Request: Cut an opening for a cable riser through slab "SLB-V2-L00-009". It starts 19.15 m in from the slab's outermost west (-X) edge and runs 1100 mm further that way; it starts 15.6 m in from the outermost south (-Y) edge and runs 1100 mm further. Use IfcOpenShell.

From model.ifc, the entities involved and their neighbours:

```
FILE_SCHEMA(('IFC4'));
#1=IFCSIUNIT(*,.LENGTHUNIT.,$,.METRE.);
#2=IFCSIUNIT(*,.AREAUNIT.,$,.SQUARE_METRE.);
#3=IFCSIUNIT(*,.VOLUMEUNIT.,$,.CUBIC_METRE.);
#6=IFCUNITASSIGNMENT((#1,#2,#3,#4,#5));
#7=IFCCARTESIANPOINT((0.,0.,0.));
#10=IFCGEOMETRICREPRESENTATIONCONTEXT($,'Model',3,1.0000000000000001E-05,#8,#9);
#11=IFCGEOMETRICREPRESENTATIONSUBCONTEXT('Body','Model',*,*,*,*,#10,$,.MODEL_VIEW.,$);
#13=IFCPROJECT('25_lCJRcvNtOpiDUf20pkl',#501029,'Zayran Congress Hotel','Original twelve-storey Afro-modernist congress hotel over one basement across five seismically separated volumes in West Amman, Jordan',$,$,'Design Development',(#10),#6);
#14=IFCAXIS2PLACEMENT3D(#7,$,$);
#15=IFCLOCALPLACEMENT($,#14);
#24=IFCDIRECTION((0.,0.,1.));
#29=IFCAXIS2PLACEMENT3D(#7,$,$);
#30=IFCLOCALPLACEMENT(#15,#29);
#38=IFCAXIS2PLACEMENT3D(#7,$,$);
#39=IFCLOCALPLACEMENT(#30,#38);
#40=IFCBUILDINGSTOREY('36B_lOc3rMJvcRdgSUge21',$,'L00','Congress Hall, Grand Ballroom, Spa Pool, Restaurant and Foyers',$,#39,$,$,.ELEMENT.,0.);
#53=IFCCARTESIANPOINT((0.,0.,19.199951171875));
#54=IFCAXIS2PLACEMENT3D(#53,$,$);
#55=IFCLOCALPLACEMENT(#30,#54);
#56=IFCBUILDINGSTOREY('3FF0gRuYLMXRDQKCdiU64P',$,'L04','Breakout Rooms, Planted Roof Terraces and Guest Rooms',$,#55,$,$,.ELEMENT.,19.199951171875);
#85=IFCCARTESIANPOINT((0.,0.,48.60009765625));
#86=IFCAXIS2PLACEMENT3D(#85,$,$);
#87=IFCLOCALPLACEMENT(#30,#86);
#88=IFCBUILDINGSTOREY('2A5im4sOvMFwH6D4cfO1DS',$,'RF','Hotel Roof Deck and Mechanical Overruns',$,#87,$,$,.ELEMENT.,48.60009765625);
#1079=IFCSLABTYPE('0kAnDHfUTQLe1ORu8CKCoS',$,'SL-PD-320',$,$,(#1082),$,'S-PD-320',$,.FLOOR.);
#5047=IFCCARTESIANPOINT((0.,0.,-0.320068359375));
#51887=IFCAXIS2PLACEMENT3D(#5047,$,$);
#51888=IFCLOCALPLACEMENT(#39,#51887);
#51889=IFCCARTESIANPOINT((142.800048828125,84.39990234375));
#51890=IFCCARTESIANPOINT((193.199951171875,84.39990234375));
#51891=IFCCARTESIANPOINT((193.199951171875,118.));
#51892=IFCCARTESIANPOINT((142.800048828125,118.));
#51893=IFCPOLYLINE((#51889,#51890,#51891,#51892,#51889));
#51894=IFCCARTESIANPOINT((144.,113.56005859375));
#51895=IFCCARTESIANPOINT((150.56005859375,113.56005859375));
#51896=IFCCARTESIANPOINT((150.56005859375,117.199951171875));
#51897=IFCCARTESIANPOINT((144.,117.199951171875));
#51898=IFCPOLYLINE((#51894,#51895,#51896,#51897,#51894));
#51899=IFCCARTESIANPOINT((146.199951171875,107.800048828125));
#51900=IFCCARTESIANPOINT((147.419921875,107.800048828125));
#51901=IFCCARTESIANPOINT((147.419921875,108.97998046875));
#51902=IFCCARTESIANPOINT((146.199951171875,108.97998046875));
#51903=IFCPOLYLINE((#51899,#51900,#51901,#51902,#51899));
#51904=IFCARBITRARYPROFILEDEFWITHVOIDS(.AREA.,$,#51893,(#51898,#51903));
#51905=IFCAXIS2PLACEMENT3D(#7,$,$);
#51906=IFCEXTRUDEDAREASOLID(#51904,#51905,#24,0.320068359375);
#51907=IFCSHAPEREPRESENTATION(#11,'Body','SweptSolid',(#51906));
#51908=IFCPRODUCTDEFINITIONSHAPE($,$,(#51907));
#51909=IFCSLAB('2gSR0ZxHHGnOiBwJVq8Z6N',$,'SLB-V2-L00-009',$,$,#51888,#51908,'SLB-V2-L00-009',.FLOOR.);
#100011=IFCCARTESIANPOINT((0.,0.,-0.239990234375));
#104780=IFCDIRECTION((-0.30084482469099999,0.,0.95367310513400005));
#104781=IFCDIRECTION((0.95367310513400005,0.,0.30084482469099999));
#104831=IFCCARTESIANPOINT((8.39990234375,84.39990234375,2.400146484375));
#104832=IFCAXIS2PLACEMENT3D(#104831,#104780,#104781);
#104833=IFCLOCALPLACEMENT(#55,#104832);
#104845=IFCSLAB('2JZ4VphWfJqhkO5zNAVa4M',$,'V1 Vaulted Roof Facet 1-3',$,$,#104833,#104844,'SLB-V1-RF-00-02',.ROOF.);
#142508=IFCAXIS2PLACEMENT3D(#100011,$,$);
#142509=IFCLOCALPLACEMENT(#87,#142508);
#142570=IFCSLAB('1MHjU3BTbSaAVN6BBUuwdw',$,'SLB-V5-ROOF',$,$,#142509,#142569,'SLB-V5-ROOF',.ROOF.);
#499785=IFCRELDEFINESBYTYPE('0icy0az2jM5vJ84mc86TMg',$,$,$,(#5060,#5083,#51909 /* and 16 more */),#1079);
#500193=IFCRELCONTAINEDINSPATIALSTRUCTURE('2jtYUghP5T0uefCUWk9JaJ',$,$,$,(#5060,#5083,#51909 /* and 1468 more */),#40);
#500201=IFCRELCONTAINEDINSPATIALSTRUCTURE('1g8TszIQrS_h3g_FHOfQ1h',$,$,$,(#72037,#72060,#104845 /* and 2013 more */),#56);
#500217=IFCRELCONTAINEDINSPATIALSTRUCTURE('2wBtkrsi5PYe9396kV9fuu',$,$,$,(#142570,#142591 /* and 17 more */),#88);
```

```python
import numpy as np
import ifcopenshell
import ifcopenshell.api.feature
import ifcopenshell.api.geometry
import ifcopenshell.api.root
import ifcopenshell.geom
import ifcopenshell.util.placement
import ifcopenshell.util.representation
import ifcopenshell.util.shape
import ifcopenshell.util.unit

model = ifcopenshell.open("model.ifc")
unit_scale = ifcopenshell.util.unit.calculate_unit_scale(model)
settings = ifcopenshell.geom.settings()


def volume(element):
    """Net volume in cubic metres, openings subtracted."""
    shape = ifcopenshell.geom.create_shape(settings, element)
    return ifcopenshell.util.shape.get_volume(shape.geometry)


slab = model.by_guid("2gSR0ZxHHGnOiBwJVq8Z6N")
before = volume(slab)

# Extent in the slab's own axes, in metres. The edges named are its -X and -Y sides.
slab_shape = ifcopenshell.geom.create_shape(settings, slab)
vertices = ifcopenshell.util.shape.get_vertices(slab_shape.geometry)
x_min, y_min, bottom = vertices.min(axis=0)
top = vertices[:, 2].max()

opening = ifcopenshell.api.root.create_entity(model, ifc_class="IfcOpeningElement", name="Cable riser opening", predefined_type="OPENING")
context = ifcopenshell.util.representation.get_context(model, "Model", "Body", "MODEL_VIEW")
width, depth = 1.1, 1.1
outline = [(0.0, 0.0), (width, 0.0), (width, depth), (0.0, depth), (0.0, 0.0)]
# Overshoot both faces by 50 mm so the cut is clean.
shape = ifcopenshell.api.geometry.add_slab_representation(
    model, context=context, depth=top - bottom + 0.1, polyline=outline
)
ifcopenshell.api.geometry.assign_representation(model, product=opening, representation=shape)

matrix = ifcopenshell.util.placement.get_local_placement(slab.ObjectPlacement)
matrix[:, 3] = matrix @ np.append(np.array([x_min + 19.15, y_min + 15.6, bottom - 0.05]) / unit_scale, 1.0)
ifcopenshell.api.geometry.edit_object_placement(model, product=opening, matrix=matrix, is_si=False)
ifcopenshell.api.feature.add_feature(model, feature=opening, element=slab)

after = volume(slab)

print(f"slab volume {before:.3f} -> {after:.3f} m3")

model.write("model_rev.ifc")
```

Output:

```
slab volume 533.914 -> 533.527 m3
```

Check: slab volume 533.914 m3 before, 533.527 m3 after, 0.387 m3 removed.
